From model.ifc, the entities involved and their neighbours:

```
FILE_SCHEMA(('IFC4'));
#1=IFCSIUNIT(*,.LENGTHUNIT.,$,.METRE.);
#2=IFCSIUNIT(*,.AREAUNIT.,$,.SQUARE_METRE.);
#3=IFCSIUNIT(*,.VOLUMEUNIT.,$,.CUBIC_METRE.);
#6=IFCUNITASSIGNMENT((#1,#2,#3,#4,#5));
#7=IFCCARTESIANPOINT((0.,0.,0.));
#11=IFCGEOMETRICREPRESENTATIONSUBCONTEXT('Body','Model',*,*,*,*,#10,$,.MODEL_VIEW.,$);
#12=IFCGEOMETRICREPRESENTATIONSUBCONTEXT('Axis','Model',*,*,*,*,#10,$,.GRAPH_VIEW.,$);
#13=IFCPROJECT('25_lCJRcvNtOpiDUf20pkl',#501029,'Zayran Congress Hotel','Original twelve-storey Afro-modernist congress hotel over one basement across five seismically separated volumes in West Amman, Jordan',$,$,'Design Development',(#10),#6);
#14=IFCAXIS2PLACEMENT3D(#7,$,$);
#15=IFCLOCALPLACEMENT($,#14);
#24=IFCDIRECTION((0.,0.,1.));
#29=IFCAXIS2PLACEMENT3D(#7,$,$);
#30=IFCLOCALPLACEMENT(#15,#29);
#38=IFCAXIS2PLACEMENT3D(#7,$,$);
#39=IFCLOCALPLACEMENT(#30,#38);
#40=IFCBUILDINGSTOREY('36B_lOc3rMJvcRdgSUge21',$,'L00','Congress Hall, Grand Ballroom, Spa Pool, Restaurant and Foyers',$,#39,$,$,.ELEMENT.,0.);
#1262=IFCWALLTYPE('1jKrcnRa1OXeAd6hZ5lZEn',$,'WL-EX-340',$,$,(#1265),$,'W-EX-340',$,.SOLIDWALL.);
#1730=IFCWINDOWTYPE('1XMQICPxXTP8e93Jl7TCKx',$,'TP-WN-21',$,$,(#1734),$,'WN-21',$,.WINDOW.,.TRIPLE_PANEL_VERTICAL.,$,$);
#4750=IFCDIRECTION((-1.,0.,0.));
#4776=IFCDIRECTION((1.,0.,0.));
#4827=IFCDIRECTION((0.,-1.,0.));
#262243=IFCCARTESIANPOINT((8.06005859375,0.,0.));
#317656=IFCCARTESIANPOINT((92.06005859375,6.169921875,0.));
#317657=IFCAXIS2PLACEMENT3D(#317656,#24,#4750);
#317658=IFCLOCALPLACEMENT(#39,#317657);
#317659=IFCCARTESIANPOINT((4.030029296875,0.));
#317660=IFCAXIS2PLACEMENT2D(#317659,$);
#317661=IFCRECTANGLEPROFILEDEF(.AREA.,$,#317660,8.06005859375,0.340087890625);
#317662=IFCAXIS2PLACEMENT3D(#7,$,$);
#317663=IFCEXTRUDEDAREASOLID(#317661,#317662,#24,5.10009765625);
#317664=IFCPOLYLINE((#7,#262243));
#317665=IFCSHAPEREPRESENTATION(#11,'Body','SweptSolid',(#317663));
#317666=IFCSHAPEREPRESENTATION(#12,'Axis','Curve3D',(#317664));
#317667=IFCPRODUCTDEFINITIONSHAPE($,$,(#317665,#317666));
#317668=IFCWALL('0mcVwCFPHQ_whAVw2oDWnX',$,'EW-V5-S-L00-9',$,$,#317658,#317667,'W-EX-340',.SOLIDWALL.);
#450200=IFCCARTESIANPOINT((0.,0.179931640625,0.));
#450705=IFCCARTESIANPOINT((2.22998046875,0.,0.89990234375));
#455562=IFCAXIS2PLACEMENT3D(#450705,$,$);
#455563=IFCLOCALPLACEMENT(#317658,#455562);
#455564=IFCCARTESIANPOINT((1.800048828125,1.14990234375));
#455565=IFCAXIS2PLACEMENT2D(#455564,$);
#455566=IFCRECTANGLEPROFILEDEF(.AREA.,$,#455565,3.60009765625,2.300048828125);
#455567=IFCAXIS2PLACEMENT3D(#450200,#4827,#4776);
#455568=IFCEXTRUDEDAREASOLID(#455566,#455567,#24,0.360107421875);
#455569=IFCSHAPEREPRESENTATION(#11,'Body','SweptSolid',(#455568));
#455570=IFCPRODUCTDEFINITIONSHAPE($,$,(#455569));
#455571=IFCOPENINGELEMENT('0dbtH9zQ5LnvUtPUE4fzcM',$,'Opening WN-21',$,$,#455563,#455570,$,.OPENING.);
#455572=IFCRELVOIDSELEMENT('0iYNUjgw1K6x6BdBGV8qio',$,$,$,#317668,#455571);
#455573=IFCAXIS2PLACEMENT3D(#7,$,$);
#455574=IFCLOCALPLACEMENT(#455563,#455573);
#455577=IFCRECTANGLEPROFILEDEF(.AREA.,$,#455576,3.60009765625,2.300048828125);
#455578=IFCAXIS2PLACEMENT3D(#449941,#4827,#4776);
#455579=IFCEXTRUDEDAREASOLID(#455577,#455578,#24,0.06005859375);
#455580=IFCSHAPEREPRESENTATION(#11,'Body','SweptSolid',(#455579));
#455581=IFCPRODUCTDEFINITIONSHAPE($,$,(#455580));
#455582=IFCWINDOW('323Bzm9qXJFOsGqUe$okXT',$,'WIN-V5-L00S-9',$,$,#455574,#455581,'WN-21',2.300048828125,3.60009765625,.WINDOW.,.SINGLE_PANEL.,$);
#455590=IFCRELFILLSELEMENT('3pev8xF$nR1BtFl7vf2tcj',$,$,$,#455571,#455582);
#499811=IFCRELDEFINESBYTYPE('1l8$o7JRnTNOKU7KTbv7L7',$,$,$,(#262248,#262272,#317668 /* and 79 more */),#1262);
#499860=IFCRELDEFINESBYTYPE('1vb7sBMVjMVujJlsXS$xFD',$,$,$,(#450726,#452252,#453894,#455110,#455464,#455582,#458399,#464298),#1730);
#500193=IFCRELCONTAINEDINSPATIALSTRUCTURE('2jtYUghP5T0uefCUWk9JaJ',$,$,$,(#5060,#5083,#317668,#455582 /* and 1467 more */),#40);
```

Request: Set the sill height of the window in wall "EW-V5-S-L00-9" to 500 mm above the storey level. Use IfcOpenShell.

```python
import numpy as np
import ifcopenshell
import ifcopenshell.api.geometry
import ifcopenshell.geom
import ifcopenshell.util.element
import ifcopenshell.util.placement
import ifcopenshell.util.shape
import ifcopenshell.util.unit

model = ifcopenshell.open("model.ifc")
unit_scale = ifcopenshell.util.unit.calculate_unit_scale(model)

window = model.by_guid("323Bzm9qXJFOsGqUe$okXT")
opening = window.FillsVoids[0].RelatingOpeningElement
storey = ifcopenshell.util.element.get_container(window, ifc_class="IfcBuildingStorey")
level = ifcopenshell.util.placement.get_local_placement(storey.ObjectPlacement)[2, 3]

# The opening's origin need not be at the sill, so measure its lowest point.
shape = ifcopenshell.geom.create_shape(ifcopenshell.geom.settings(), opening)
bottom = ifcopenshell.util.shape.get_shape_bottom_elevation(shape, shape.geometry) / unit_scale
dz = level + 0.5 / unit_scale - bottom

shift = np.array([0.0, 0.0, dz])
# The window is placed relative to its opening, so it follows when the opening moves.
matrix = ifcopenshell.util.placement.get_local_placement(opening.ObjectPlacement)
matrix[:3, 3] += shift
ifcopenshell.api.geometry.edit_object_placement(
    model, product=opening, matrix=matrix, is_si=False, should_transform_children=True
)

print(f"moved by {dz * unit_scale:+.3f} m")

model.write("model_updated.ifc")
```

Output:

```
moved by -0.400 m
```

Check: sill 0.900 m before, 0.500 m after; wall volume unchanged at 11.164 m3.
